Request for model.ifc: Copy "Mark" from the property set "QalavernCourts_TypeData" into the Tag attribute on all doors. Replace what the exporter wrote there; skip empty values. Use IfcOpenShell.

First a look at what the model holds.

```python
import ifcopenshell
import ifcopenshell.util.element

model = ifcopenshell.open("model.ifc")
print(model.schema)
doors = model.by_type("IfcDoor")
print(len(doors), "doors")
for e in doors[:8]:
    source = ifcopenshell.util.element.get_pset(e, "QalavernCourts_TypeData", "Mark")
    target = e.Tag
    print(e.id(), repr(source), repr(target), sep=" | ")
```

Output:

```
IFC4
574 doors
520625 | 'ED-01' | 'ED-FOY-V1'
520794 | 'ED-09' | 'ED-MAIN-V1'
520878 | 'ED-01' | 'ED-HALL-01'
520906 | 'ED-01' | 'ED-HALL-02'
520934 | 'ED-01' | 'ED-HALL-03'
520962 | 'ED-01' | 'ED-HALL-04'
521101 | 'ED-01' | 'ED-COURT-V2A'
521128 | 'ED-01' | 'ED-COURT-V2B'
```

```python
import ifcopenshell
import ifcopenshell.util.element

model = ifcopenshell.open("model.ifc")

count = 0
for e in model.by_type("IfcDoor"):
    value = ifcopenshell.util.element.get_pset(e, "QalavernCourts_TypeData", "Mark")
    current = e.Tag
    if not value or not value.strip() or current == value:
        continue
    e.Tag = value
    count += 1

print(count, "doors updated")

model.write("model_v2.ifc")
```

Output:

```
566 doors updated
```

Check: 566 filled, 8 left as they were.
